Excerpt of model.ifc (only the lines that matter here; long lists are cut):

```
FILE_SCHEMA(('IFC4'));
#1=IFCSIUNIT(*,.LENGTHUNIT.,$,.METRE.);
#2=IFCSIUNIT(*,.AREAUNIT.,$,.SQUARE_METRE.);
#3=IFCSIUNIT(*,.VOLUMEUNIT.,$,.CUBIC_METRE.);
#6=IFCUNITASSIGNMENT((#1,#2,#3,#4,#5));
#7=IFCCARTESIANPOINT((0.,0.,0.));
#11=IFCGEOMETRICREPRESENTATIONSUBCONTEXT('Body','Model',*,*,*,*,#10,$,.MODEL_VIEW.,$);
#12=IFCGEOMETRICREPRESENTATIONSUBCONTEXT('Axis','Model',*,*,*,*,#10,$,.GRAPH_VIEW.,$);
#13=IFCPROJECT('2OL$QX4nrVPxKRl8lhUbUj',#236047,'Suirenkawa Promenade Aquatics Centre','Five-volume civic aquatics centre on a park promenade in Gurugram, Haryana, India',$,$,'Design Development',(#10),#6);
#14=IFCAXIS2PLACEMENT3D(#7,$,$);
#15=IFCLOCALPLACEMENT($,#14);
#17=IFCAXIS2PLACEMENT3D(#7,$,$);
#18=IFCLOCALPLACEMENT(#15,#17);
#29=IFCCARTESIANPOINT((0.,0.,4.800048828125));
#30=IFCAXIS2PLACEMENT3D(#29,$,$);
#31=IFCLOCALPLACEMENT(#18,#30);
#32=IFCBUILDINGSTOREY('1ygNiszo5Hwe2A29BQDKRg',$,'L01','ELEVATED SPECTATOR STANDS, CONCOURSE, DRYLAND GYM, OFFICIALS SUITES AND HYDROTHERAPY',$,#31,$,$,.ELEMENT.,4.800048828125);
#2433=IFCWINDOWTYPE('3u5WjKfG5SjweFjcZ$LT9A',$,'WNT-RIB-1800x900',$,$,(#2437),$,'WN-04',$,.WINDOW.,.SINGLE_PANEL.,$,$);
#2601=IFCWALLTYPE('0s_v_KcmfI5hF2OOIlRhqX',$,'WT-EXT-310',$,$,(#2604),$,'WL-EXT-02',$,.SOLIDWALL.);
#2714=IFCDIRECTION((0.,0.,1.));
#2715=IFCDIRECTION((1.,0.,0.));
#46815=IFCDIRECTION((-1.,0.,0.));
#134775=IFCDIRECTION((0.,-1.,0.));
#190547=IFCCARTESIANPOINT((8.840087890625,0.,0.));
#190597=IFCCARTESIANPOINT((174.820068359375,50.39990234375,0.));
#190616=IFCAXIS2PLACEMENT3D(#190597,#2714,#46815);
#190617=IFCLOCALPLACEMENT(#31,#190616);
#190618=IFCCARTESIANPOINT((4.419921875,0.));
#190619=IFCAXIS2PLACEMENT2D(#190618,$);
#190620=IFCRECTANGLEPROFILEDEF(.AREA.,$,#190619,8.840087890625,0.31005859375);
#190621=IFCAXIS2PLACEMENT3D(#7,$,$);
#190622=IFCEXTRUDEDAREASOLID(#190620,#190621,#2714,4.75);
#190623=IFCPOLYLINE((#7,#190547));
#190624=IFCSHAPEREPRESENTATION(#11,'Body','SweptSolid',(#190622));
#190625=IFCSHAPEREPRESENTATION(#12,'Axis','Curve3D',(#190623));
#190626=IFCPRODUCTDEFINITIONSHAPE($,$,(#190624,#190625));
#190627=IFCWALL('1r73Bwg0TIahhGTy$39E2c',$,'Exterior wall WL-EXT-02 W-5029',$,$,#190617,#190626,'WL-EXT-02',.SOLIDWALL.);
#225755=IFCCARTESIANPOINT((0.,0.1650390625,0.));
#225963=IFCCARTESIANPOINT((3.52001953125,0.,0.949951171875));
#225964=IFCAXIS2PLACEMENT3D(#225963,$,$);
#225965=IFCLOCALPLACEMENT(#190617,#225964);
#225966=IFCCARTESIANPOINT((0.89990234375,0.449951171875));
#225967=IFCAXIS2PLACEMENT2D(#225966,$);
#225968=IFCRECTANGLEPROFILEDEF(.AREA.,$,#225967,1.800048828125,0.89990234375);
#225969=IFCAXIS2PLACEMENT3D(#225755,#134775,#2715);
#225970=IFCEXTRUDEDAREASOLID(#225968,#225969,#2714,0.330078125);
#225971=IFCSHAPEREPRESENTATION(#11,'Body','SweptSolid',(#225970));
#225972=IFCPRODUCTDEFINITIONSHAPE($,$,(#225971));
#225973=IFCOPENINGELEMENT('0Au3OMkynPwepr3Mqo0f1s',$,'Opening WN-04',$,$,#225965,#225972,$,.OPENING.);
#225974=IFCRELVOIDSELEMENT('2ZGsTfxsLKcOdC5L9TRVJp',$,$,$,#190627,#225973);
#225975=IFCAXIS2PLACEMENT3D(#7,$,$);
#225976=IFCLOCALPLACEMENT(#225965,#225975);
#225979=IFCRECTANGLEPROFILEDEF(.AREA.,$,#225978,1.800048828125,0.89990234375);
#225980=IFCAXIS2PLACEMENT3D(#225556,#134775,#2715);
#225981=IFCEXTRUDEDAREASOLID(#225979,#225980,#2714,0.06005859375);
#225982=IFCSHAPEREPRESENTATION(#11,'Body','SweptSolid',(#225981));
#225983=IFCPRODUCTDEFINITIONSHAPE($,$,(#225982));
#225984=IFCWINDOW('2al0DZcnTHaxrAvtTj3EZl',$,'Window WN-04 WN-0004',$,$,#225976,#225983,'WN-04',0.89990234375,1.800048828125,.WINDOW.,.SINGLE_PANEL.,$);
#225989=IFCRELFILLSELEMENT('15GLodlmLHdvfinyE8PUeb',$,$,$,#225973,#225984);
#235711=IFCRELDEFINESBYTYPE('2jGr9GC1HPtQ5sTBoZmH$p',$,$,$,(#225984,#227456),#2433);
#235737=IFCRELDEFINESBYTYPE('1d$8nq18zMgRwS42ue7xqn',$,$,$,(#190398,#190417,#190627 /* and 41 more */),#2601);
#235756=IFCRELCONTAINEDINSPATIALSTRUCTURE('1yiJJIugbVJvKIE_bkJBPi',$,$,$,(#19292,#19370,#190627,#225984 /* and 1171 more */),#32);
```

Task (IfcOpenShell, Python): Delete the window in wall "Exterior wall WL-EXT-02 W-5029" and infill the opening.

```python
import ifcopenshell
import ifcopenshell.api.feature
import ifcopenshell.api.root
import ifcopenshell.geom
import ifcopenshell.util.shape

model = ifcopenshell.open("model.ifc")
settings = ifcopenshell.geom.settings()


def volume(element):
    """Net volume in cubic metres, openings subtracted."""
    shape = ifcopenshell.geom.create_shape(settings, element)
    return ifcopenshell.util.shape.get_volume(shape.geometry)


window = model.by_id(225984)
opening = window.FillsVoids[0].RelatingOpeningElement
wall = opening.VoidsElements[0].RelatingBuildingElement
before = volume(wall)

ifcopenshell.api.root.remove_product(model, product=window)
ifcopenshell.api.feature.remove_feature(model, feature=opening)

after = volume(wall)

print(f"wall volume {before:.3f} -> {after:.3f} m3")

model.write("model_v2.ifc")
```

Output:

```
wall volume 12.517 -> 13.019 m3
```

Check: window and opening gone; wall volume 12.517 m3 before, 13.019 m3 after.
